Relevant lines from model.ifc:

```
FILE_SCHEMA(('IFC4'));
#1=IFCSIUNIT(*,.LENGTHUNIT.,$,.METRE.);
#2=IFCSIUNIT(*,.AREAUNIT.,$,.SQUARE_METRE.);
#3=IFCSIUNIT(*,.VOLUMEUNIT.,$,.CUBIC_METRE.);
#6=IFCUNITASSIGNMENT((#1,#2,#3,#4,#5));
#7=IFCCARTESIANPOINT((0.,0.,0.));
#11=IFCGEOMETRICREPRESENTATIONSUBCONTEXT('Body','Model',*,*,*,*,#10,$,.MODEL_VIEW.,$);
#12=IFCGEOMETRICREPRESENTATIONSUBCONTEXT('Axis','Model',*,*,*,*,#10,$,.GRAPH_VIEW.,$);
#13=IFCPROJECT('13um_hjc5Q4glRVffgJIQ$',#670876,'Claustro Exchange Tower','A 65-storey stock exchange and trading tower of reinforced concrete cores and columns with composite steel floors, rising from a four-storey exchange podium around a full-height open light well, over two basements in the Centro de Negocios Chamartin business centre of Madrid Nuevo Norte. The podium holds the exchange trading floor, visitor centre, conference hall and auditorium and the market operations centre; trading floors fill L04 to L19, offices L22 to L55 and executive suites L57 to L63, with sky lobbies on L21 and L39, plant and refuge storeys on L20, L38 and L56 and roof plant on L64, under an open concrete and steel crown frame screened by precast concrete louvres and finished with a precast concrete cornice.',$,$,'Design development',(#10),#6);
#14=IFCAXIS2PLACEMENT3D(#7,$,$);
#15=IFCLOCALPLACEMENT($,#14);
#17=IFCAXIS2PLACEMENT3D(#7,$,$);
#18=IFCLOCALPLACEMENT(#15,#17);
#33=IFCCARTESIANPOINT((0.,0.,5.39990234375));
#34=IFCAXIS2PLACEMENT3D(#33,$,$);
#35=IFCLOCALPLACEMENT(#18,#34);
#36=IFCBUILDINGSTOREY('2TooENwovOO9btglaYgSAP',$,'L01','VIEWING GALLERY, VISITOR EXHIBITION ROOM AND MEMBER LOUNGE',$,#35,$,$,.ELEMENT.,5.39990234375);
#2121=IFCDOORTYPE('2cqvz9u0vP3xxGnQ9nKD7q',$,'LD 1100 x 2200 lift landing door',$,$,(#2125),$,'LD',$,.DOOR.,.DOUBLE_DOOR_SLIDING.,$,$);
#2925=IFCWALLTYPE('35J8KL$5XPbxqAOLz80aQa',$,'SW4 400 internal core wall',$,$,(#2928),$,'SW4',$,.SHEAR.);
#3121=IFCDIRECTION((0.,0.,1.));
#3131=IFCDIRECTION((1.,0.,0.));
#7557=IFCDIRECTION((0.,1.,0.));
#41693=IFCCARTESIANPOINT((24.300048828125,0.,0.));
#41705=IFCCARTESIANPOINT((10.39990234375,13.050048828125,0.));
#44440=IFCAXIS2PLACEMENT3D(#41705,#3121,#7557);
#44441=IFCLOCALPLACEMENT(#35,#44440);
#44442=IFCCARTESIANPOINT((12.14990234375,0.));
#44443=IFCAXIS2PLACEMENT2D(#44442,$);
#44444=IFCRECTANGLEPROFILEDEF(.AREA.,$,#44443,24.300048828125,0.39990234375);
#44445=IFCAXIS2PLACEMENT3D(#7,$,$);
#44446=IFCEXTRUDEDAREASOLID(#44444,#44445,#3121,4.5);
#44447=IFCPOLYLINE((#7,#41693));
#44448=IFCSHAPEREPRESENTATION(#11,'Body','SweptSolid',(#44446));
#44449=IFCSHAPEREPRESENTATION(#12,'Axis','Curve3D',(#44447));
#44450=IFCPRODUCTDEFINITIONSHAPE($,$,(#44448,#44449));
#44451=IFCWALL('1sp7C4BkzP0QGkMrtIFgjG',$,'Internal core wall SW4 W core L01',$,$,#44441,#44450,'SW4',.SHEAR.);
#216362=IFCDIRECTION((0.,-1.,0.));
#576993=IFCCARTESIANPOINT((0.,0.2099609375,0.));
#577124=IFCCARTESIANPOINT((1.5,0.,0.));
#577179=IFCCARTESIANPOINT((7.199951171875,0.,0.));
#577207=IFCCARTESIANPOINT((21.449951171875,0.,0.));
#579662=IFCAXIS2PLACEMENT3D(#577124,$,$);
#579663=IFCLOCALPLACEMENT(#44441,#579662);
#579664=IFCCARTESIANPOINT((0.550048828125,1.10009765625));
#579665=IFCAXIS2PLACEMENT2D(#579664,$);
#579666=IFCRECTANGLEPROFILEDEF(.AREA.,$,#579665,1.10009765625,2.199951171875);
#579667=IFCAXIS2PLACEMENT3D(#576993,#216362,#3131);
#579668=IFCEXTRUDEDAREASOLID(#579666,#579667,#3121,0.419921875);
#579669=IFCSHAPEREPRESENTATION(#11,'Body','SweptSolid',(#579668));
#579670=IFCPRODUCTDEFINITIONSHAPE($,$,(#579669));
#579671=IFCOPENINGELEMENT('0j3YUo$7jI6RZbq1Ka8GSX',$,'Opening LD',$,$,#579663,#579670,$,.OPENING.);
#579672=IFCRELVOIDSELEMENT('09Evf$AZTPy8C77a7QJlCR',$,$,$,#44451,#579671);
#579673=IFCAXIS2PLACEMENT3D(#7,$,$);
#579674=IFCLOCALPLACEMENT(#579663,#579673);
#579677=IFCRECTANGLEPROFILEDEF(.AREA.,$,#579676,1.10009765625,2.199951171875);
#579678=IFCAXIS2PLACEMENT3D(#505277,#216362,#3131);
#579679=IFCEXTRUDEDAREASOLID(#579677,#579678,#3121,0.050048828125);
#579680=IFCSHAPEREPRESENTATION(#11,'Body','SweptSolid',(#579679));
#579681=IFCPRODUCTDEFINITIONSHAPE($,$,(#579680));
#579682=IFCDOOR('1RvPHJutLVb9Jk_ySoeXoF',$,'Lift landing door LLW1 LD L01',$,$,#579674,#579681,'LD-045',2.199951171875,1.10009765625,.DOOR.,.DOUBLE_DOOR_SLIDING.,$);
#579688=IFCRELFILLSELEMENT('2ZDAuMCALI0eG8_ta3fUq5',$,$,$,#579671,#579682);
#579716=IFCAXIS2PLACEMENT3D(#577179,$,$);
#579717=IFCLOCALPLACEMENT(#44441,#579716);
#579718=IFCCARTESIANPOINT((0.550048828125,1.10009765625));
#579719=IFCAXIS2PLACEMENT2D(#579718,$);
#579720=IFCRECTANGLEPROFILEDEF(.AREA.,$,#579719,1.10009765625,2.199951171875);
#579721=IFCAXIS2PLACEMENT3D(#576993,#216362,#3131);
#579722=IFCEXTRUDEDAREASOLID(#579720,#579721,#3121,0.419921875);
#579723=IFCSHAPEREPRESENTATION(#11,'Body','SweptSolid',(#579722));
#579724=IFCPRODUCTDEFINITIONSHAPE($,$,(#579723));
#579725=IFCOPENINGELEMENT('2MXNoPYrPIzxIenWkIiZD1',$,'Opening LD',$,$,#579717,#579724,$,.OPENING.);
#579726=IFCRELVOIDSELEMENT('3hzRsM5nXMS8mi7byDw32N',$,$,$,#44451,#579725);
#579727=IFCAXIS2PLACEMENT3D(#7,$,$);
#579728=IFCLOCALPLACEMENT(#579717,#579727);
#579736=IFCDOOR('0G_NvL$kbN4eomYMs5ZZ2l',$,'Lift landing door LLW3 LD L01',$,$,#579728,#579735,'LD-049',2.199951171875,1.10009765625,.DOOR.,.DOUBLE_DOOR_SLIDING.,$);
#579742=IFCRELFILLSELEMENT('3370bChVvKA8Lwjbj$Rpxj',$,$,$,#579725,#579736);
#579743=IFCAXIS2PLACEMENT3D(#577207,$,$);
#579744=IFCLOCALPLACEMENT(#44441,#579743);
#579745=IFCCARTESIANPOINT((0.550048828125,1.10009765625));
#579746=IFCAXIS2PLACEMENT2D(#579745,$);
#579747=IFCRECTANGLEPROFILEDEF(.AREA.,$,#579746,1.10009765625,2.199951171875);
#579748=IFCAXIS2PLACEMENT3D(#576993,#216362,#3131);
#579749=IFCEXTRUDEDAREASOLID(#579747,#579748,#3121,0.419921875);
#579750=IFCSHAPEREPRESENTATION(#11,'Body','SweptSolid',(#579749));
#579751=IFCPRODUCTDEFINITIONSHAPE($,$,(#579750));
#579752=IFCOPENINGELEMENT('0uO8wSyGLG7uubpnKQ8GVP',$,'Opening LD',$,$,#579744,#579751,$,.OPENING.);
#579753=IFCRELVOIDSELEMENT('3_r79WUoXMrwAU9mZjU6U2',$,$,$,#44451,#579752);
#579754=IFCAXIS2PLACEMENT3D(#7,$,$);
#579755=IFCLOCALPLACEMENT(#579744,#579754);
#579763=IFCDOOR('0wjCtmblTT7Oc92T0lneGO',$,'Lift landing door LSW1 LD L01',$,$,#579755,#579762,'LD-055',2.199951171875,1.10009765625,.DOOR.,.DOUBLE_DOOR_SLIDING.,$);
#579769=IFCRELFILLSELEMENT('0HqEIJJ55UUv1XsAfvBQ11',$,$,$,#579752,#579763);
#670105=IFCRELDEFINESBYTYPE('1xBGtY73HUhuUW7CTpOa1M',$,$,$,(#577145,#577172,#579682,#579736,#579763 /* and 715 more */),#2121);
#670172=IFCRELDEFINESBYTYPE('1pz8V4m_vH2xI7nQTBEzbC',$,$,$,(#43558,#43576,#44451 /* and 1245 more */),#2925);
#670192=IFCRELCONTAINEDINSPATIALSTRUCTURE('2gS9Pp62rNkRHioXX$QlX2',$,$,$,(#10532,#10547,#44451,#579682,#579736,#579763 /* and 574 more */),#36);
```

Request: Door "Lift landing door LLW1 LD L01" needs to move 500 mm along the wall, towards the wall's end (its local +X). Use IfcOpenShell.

```python
import ifcopenshell
import ifcopenshell.api.geometry
import ifcopenshell.util.placement
import ifcopenshell.util.unit

model = ifcopenshell.open("model.ifc")
unit_scale = ifcopenshell.util.unit.calculate_unit_scale(model)

door = model.by_id(579682)
opening = door.FillsVoids[0].RelatingOpeningElement
wall = opening.VoidsElements[0].RelatingBuildingElement

wall_matrix = ifcopenshell.util.placement.get_local_placement(wall.ObjectPlacement)
shift = wall_matrix[:3, 0] * 0.5 / unit_scale
before = ifcopenshell.util.placement.get_local_placement(door.ObjectPlacement)[:3, 3].copy()

# The door is placed relative to its opening, so it follows when the opening moves.
matrix = ifcopenshell.util.placement.get_local_placement(opening.ObjectPlacement)
matrix[:3, 3] += shift
ifcopenshell.api.geometry.edit_object_placement(
    model, product=opening, matrix=matrix, is_si=False, should_transform_children=True
)

after = ifcopenshell.util.placement.get_local_placement(door.ObjectPlacement)[:3, 3]
print("door moved by", (after - before).round(3) + 0.0)

model.write("model_rev.ifc")
```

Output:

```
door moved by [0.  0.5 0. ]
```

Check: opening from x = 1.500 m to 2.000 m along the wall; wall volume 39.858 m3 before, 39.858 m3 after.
